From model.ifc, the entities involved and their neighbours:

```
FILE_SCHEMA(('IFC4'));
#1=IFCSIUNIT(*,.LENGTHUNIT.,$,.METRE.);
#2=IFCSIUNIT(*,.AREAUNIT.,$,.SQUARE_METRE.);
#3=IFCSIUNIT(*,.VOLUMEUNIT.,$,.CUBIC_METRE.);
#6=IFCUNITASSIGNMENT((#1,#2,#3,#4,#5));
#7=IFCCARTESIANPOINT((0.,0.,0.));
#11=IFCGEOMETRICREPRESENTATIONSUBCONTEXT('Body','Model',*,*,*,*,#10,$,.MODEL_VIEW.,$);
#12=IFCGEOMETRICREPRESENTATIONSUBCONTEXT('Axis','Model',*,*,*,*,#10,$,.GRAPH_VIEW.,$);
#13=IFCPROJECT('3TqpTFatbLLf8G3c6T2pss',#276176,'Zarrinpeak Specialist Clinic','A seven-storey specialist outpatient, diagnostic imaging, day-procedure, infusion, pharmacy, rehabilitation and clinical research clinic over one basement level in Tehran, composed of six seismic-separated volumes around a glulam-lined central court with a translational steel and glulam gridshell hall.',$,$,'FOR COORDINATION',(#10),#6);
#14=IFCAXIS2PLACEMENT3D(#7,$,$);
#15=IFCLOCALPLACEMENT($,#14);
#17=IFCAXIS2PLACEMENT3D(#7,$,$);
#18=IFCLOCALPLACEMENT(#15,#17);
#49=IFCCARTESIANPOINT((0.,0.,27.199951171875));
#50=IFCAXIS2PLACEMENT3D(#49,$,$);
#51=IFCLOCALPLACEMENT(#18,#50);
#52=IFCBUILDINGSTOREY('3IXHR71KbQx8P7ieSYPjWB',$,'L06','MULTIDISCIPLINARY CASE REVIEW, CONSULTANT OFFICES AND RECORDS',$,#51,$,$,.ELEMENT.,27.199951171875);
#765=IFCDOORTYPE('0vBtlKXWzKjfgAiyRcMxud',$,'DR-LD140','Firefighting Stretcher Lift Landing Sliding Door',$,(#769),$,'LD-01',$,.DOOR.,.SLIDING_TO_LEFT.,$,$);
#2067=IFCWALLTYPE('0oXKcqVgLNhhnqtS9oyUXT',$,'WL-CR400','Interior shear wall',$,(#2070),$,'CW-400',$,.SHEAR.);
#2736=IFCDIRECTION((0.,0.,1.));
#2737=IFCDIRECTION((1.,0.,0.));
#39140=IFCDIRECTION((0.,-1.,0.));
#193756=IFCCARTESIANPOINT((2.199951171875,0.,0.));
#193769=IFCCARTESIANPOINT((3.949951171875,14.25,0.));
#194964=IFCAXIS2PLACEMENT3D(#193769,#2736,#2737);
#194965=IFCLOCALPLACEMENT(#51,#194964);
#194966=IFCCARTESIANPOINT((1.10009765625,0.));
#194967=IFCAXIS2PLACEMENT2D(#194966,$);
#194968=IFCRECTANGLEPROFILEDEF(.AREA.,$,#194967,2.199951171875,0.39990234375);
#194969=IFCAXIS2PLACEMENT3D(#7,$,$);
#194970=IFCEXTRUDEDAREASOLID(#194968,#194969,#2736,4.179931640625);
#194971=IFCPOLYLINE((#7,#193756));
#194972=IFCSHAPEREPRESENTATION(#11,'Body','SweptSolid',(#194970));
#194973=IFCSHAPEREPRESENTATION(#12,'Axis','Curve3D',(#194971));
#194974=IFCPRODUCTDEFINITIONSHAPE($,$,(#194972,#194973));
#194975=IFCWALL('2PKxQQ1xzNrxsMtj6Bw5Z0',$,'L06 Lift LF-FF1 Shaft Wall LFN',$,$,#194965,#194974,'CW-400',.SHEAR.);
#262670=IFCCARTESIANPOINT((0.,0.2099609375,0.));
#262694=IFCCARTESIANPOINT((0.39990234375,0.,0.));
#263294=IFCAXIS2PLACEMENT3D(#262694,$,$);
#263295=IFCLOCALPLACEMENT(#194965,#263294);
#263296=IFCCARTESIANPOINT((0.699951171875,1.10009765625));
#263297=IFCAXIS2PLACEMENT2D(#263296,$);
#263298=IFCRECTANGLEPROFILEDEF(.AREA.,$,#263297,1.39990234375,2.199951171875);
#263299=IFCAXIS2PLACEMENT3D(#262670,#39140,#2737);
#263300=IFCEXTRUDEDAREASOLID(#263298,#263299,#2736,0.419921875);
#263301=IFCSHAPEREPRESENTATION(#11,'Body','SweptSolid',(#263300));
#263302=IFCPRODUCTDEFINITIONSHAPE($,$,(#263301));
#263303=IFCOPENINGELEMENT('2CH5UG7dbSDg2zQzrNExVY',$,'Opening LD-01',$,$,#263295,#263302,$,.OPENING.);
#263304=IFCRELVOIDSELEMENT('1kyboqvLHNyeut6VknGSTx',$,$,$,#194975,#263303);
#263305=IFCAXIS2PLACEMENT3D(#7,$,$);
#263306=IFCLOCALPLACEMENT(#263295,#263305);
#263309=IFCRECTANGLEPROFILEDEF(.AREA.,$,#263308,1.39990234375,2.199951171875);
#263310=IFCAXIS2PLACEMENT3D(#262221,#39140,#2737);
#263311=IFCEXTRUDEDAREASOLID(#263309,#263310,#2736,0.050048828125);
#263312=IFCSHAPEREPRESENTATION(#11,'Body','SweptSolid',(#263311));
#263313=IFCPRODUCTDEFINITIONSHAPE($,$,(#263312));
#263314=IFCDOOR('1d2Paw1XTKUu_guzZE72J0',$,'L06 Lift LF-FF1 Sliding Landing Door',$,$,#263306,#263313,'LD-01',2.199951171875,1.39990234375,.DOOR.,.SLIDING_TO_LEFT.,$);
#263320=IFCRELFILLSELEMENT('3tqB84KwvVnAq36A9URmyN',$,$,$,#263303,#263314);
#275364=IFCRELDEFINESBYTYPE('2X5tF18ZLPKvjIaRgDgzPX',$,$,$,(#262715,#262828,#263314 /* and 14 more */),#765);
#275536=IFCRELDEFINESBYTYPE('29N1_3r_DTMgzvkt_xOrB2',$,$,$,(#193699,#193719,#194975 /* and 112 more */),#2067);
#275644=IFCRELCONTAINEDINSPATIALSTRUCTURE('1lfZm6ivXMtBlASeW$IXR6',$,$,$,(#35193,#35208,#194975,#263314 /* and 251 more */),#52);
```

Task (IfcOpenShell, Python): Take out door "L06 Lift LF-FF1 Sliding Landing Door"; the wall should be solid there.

```python
import ifcopenshell
import ifcopenshell.api.feature
import ifcopenshell.api.root
import ifcopenshell.geom
import ifcopenshell.util.shape

model = ifcopenshell.open("model.ifc")
settings = ifcopenshell.geom.settings()


def volume(element):
    """Net volume in cubic metres, openings subtracted."""
    shape = ifcopenshell.geom.create_shape(settings, element)
    return ifcopenshell.util.shape.get_volume(shape.geometry)


door = model.by_guid("1d2Paw1XTKUu_guzZE72J0")
opening = door.FillsVoids[0].RelatingOpeningElement
wall = opening.VoidsElements[0].RelatingBuildingElement
before = volume(wall)

ifcopenshell.api.root.remove_product(model, product=door)
ifcopenshell.api.feature.remove_feature(model, feature=opening)

after = volume(wall)

print(f"wall volume {before:.3f} -> {after:.3f} m3")

model.write("model_updated.ifc")
```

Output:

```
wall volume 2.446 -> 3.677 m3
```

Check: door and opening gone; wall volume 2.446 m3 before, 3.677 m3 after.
